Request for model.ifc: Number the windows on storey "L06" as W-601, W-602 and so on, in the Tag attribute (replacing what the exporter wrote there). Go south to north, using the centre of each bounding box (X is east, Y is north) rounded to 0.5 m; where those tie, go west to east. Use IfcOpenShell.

First a look at what the model holds.

```python
import ifcopenshell
import ifcopenshell.util.element
import ifcopenshell.util.placement

model = ifcopenshell.open("model.ifc")
print(model.schema)
storey = next(s for s in model.by_type("IfcBuildingStorey") if s.Name == "L06")
windows = [e for e in ifcopenshell.util.element.get_decomposition(storey) if e.is_a("IfcWindow")]
for e in sorted(windows, key=lambda e: e.id()):
    origin = ifcopenshell.util.placement.get_local_placement(e.ObjectPlacement)[:3, 3]
    print(e.id(), e.Tag, e.Name, origin.round(2) + 0.0, sep=" | ")
```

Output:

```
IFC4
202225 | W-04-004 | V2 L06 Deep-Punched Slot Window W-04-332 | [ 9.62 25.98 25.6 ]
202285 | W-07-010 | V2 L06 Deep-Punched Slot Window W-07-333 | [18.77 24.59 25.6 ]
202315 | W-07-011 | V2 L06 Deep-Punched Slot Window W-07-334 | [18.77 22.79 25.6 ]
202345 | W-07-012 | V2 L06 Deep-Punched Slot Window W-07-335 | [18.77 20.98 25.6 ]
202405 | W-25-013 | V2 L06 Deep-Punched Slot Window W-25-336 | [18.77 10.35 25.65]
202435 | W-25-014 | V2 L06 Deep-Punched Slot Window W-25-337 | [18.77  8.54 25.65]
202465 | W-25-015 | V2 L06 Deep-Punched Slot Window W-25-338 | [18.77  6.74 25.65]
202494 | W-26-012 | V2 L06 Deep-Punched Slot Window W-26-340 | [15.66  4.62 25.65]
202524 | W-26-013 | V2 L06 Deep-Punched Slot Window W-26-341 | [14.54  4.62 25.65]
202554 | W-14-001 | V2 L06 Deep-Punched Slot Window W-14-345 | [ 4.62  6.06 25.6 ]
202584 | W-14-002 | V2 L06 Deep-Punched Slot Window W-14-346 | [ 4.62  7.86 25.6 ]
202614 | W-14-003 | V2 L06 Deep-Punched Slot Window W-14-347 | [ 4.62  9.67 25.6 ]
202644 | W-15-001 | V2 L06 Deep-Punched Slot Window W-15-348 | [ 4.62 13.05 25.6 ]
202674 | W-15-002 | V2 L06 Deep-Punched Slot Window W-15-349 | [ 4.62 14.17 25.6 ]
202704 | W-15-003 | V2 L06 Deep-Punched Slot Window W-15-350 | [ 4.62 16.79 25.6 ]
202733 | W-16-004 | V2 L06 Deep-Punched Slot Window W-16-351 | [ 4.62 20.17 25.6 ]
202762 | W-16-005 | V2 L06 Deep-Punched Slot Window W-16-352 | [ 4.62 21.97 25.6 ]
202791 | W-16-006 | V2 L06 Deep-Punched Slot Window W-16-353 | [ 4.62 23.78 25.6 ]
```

```python
import ifcopenshell
import ifcopenshell.geom
import ifcopenshell.util.element
import ifcopenshell.util.shape

model = ifcopenshell.open("model.ifc")
settings = ifcopenshell.geom.settings()
settings.set("use-world-coords", True)


def centre(element):
    shape = ifcopenshell.geom.create_shape(settings, element)
    return ifcopenshell.util.shape.get_bbox_centroid(shape.geometry)


storey = next(s for s in model.by_type("IfcBuildingStorey") if s.Name == "L06")
windows = [e for e in ifcopenshell.util.element.get_decomposition(storey) if e.is_a("IfcWindow")]

# Insertion points can sit at a corner or the storey origin, so sort by the geometry (in metres).
centres = {e: centre(e) for e in windows}
windows.sort(key=lambda e: (round(centres[e][1] / 0.5), centres[e][0]))

for i, e in enumerate(windows, start=1):
    number = f"W-6{i:02d}"
    e.Tag = number
    print(e.id(), number)

model.write("model_updated.ifc")
```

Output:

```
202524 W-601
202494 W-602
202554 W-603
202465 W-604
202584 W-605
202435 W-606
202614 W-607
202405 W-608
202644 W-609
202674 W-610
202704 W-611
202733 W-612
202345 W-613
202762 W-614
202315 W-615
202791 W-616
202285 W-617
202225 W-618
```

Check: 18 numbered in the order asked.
